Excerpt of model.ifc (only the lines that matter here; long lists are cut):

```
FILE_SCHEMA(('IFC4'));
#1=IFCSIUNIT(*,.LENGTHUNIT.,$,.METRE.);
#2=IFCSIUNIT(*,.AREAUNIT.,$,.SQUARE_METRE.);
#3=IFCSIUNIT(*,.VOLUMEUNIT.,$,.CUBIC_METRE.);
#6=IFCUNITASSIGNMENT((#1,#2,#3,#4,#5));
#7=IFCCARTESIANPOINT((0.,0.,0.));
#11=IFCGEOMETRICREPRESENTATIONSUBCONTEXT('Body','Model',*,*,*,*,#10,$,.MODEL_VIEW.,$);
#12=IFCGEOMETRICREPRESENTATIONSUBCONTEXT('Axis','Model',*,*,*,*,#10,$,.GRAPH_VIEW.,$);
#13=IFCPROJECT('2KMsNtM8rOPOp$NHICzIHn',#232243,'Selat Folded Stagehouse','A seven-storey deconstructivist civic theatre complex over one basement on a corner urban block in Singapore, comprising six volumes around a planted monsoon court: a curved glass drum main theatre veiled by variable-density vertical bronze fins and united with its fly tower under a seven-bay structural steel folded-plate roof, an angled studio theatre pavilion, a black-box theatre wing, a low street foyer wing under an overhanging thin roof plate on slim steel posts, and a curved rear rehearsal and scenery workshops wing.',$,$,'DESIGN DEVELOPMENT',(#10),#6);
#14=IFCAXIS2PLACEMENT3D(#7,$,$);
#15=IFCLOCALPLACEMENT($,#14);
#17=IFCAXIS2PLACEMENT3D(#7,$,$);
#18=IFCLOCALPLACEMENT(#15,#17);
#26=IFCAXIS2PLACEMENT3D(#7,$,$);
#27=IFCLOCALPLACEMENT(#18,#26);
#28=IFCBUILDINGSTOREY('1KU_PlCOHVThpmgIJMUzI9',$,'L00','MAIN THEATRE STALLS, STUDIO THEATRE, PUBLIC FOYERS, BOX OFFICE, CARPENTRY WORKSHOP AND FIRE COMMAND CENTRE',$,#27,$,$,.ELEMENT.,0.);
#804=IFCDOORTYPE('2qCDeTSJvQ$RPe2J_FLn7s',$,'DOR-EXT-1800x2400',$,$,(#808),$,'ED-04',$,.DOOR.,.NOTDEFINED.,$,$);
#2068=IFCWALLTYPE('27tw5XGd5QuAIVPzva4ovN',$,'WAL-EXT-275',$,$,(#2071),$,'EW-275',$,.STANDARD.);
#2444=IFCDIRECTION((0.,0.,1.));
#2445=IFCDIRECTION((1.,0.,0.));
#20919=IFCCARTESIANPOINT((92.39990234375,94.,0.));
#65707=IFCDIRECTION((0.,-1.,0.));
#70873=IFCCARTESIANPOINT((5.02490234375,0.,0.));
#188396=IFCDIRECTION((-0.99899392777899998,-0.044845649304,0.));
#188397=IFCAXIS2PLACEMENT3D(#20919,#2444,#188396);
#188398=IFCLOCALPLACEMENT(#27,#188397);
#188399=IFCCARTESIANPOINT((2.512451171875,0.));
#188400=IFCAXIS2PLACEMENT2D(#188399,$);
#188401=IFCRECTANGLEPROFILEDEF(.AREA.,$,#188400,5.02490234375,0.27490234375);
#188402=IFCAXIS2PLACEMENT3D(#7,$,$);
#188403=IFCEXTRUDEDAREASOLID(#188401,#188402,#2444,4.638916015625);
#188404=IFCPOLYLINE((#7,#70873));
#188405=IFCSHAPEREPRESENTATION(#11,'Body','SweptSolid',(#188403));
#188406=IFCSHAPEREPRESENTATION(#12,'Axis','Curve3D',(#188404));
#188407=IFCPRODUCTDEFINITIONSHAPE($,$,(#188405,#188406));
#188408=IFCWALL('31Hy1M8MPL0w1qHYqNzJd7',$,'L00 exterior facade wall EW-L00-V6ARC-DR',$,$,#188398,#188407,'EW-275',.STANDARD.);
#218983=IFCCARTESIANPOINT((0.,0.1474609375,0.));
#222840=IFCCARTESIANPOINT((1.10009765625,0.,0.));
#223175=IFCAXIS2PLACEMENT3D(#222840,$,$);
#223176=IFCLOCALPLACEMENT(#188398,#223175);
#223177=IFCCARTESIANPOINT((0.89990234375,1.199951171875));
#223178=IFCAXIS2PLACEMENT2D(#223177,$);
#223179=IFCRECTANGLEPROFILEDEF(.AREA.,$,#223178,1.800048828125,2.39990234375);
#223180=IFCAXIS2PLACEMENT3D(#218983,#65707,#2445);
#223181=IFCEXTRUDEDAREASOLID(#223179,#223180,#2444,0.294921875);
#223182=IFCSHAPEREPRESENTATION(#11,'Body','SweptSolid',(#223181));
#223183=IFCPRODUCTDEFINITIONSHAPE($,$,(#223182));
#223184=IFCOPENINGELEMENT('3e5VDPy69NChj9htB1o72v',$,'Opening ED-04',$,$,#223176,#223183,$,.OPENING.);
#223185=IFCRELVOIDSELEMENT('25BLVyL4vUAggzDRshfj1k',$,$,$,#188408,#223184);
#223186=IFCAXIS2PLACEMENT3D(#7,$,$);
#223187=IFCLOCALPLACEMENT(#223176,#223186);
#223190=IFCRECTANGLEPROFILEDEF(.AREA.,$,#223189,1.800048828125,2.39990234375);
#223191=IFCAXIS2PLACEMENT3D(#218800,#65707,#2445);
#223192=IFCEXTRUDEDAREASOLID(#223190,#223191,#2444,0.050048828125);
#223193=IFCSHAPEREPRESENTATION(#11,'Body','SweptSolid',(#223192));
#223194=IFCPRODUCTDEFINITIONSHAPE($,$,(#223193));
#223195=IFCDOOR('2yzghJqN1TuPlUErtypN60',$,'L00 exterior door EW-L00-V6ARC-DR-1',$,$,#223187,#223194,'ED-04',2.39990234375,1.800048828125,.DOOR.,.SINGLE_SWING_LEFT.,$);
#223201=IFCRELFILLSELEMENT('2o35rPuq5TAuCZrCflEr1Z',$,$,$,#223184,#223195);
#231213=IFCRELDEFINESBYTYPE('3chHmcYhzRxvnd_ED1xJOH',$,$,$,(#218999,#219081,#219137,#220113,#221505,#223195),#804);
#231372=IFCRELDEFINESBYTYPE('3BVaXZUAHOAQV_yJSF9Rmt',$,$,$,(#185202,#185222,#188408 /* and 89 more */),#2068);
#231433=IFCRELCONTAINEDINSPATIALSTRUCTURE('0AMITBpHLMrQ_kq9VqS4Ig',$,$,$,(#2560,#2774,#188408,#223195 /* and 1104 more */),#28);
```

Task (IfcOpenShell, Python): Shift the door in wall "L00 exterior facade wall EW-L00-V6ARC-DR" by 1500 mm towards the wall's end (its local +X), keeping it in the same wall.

```python
import ifcopenshell
import ifcopenshell.api.geometry
import ifcopenshell.util.placement
import ifcopenshell.util.unit

model = ifcopenshell.open("model.ifc")
unit_scale = ifcopenshell.util.unit.calculate_unit_scale(model)

door = model.by_guid("2yzghJqN1TuPlUErtypN60")
opening = door.FillsVoids[0].RelatingOpeningElement
wall = opening.VoidsElements[0].RelatingBuildingElement

wall_matrix = ifcopenshell.util.placement.get_local_placement(wall.ObjectPlacement)
shift = wall_matrix[:3, 0] * 1.5 / unit_scale
before = ifcopenshell.util.placement.get_local_placement(door.ObjectPlacement)[:3, 3].copy()

# The door is placed relative to its opening, so it follows when the opening moves.
matrix = ifcopenshell.util.placement.get_local_placement(opening.ObjectPlacement)
matrix[:3, 3] += shift
ifcopenshell.api.geometry.edit_object_placement(
    model, product=opening, matrix=matrix, is_si=False, should_transform_children=True
)

after = ifcopenshell.util.placement.get_local_placement(door.ObjectPlacement)[:3, 3]
print("door moved by", (after - before).round(3) + 0.0)

model.write("model_edited.ifc")
```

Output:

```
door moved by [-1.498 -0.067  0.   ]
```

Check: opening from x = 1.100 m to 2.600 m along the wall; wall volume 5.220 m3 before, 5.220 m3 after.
